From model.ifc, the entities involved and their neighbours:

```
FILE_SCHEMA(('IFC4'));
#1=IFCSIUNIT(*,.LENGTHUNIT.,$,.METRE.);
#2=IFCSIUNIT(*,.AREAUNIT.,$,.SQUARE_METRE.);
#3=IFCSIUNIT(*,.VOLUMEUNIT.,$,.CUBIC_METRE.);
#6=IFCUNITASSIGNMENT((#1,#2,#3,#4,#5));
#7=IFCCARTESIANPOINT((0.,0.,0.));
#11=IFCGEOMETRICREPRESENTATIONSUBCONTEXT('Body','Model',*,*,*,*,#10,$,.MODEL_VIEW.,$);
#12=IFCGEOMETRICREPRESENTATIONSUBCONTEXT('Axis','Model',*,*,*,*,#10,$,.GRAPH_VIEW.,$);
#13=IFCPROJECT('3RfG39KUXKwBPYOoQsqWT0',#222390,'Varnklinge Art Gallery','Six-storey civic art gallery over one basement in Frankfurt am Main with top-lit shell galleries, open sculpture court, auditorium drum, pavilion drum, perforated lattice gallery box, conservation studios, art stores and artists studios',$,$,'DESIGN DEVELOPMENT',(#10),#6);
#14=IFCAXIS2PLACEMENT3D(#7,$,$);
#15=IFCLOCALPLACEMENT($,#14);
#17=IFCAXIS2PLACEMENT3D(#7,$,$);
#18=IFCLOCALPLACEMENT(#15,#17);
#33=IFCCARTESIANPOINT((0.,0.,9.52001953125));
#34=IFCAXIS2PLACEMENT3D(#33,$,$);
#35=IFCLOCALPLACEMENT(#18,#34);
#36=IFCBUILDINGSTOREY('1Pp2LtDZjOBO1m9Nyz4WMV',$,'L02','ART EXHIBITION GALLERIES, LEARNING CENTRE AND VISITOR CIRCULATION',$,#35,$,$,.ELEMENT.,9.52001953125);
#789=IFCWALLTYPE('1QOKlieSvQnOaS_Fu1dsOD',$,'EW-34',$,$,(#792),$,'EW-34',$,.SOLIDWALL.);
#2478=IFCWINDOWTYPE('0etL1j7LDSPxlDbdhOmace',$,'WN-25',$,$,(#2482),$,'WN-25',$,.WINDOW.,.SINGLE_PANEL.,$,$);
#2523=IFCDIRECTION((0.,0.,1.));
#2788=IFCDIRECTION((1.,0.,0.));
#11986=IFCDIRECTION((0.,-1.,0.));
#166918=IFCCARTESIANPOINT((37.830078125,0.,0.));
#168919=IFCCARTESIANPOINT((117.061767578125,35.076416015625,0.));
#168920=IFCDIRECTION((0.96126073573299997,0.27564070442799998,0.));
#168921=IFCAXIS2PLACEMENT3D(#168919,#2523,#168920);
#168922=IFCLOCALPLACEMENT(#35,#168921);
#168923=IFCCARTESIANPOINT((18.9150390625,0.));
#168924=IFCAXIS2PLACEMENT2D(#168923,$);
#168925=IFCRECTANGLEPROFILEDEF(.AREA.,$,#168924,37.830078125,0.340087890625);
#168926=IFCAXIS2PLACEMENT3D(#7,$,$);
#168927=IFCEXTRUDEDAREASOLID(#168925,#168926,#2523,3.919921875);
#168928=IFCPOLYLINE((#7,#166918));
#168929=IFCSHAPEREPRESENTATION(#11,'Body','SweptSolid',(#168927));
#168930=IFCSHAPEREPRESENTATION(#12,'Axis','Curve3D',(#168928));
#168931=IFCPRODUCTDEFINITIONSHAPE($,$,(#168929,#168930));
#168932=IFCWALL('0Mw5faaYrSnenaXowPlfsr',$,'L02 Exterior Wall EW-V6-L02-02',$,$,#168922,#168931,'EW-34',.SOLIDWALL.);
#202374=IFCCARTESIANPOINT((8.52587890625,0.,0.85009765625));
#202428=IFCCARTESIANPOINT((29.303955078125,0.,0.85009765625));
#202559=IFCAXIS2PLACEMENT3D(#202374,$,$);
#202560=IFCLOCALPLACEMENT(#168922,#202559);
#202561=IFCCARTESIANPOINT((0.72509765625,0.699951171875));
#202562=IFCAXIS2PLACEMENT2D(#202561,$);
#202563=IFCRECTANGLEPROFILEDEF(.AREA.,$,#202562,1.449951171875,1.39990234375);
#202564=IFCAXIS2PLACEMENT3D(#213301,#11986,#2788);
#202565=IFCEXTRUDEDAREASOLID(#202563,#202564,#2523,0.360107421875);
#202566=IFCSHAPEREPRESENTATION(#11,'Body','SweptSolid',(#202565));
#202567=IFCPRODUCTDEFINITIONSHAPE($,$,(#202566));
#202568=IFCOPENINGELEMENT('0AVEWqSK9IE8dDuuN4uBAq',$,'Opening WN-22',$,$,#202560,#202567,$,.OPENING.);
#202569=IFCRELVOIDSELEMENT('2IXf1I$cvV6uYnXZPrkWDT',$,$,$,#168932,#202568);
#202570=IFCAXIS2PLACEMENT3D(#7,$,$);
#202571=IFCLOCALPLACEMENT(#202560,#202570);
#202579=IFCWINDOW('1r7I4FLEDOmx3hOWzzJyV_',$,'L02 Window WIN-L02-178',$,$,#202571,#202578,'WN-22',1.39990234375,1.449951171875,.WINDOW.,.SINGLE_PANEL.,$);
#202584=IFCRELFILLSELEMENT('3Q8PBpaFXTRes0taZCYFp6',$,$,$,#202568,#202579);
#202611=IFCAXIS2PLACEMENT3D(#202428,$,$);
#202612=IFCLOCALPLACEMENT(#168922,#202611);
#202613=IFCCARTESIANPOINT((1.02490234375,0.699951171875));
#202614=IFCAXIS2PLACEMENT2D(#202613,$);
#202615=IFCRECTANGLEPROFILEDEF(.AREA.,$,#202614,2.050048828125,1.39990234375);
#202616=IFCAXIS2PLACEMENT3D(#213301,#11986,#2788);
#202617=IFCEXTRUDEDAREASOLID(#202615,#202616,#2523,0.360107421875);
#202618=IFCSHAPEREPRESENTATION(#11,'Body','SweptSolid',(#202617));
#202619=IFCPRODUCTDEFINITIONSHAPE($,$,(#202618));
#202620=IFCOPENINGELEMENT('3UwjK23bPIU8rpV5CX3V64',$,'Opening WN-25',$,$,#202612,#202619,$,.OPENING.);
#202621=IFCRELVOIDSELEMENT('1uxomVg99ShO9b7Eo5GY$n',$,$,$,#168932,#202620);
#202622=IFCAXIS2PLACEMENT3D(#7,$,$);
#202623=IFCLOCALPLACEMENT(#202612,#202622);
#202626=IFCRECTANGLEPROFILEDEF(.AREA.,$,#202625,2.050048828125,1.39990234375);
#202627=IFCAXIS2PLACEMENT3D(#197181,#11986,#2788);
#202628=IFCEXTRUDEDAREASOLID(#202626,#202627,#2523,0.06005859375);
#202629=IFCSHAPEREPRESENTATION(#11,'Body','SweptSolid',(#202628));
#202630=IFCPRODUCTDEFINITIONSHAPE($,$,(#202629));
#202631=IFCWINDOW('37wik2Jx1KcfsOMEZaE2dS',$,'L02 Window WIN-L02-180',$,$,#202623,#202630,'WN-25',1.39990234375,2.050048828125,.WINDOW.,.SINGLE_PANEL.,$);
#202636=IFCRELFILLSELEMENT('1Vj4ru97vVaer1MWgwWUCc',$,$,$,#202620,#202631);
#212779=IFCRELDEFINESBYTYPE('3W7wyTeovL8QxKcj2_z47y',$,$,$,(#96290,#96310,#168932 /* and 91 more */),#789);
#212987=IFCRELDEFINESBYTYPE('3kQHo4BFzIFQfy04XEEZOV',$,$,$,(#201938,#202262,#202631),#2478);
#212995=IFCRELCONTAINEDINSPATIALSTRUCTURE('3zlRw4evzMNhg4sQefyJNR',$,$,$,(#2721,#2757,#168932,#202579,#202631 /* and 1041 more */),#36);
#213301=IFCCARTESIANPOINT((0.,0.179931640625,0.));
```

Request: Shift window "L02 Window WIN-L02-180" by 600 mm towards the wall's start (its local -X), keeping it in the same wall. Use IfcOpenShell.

```python
import ifcopenshell
import ifcopenshell.api.geometry
import ifcopenshell.util.placement
import ifcopenshell.util.unit

model = ifcopenshell.open("model.ifc")
unit_scale = ifcopenshell.util.unit.calculate_unit_scale(model)

window = model.by_guid("37wik2Jx1KcfsOMEZaE2dS")
opening = window.FillsVoids[0].RelatingOpeningElement
wall = opening.VoidsElements[0].RelatingBuildingElement

wall_matrix = ifcopenshell.util.placement.get_local_placement(wall.ObjectPlacement)
shift = wall_matrix[:3, 0] * -0.6 / unit_scale
before = ifcopenshell.util.placement.get_local_placement(window.ObjectPlacement)[:3, 3].copy()

# The window is placed relative to its opening, so it follows when the opening moves.
matrix = ifcopenshell.util.placement.get_local_placement(opening.ObjectPlacement)
matrix[:3, 3] += shift
ifcopenshell.api.geometry.edit_object_placement(
    model, product=opening, matrix=matrix, is_si=False, should_transform_children=True
)

after = ifcopenshell.util.placement.get_local_placement(window.ObjectPlacement)[:3, 3]
print("window moved by", (after - before).round(3) + 0.0)

model.write("model_v2.ifc")
```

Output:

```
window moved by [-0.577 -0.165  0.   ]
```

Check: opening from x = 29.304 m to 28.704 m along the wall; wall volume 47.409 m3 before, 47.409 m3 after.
